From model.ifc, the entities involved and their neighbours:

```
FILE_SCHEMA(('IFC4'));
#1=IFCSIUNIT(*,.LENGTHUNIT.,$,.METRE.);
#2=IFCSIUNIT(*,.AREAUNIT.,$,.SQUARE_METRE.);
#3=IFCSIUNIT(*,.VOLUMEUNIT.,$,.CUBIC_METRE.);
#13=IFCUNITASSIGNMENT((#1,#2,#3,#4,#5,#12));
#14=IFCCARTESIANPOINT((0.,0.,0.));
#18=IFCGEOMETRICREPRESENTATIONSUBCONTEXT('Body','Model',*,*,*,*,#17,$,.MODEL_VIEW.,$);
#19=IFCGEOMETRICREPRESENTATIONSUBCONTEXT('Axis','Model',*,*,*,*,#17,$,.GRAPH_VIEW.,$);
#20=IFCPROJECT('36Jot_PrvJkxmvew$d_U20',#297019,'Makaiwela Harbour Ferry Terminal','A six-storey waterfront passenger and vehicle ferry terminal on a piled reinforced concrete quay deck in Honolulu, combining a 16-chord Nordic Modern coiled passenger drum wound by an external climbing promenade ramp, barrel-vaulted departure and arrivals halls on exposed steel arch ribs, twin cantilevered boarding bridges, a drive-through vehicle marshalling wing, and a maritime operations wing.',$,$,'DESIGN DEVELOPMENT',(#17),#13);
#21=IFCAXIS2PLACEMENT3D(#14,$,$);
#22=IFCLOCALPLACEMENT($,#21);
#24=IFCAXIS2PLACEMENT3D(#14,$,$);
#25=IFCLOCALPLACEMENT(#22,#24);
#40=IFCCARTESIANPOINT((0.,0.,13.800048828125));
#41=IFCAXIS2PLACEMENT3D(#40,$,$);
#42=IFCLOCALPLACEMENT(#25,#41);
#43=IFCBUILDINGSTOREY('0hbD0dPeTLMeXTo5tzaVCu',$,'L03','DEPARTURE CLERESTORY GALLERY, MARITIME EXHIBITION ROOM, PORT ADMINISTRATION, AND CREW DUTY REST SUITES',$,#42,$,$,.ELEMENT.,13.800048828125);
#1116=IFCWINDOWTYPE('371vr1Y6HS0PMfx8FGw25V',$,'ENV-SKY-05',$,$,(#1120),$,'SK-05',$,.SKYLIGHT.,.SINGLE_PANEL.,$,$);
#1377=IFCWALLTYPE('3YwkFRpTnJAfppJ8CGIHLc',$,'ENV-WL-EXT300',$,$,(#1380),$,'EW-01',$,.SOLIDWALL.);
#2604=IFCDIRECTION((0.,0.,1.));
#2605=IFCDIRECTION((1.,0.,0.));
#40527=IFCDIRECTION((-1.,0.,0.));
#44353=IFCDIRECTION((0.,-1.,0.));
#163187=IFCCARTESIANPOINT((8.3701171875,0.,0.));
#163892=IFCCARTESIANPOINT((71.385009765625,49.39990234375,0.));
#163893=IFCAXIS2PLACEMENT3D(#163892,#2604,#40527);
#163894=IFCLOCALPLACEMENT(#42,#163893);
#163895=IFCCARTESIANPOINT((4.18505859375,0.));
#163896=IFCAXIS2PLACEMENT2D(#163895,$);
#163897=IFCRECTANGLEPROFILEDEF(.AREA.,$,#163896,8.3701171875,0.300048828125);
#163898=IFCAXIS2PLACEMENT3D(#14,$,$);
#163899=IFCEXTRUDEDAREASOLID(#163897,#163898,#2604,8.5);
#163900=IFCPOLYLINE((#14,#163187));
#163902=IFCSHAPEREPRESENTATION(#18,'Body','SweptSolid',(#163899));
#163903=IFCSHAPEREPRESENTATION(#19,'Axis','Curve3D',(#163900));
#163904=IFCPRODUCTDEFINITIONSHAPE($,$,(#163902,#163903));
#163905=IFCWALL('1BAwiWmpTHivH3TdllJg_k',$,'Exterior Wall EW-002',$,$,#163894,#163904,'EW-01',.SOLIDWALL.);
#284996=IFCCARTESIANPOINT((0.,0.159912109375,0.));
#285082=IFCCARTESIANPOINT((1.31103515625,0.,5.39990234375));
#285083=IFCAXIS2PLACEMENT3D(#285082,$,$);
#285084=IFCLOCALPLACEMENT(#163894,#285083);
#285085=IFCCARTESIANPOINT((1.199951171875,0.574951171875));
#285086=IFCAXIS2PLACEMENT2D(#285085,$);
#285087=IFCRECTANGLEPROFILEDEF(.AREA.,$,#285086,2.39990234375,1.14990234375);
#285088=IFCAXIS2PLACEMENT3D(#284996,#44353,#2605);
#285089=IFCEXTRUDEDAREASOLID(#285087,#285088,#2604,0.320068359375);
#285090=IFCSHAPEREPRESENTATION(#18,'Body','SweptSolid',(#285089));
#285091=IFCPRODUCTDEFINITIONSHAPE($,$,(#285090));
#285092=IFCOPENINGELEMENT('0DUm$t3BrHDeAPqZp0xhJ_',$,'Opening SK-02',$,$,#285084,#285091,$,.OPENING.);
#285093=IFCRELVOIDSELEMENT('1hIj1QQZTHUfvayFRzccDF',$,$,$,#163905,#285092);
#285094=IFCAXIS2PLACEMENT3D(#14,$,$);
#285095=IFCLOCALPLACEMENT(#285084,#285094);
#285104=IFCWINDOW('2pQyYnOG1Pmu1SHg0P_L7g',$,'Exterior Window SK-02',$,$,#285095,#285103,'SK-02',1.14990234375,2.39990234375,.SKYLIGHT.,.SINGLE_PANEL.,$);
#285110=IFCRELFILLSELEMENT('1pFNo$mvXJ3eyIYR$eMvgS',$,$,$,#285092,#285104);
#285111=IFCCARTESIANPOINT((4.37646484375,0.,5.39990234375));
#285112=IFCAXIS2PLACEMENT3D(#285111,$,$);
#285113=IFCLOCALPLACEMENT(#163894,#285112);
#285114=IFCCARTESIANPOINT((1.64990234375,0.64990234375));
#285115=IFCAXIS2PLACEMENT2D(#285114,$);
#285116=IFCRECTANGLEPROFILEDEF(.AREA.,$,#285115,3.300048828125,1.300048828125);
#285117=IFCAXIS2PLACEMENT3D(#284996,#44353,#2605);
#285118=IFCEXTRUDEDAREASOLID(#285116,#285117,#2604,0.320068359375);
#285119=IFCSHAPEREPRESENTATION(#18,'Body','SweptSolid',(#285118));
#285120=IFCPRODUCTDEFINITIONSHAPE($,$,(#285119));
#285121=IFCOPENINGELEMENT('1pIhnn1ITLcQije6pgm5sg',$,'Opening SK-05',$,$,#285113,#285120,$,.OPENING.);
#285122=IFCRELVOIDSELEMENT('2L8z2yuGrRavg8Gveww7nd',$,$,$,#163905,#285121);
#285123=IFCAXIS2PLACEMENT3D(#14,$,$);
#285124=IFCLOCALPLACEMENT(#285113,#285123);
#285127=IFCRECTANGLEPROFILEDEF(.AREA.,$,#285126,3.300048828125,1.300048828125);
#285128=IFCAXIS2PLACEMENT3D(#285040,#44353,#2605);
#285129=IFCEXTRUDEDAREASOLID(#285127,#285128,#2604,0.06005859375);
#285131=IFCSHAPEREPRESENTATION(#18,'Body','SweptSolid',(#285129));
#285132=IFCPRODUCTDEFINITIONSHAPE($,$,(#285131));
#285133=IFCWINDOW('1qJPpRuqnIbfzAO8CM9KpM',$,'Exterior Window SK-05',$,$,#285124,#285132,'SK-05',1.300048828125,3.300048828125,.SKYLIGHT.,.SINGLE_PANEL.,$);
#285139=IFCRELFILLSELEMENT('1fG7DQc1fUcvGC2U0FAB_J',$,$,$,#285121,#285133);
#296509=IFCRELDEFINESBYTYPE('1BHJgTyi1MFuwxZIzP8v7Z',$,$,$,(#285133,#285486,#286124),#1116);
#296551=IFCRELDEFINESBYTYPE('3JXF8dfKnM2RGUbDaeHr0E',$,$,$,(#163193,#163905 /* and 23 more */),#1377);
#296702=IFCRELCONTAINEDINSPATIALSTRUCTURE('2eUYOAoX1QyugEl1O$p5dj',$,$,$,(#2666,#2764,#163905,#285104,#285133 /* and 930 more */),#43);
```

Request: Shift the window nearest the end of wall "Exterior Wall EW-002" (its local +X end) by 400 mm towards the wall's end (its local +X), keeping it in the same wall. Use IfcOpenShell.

```python
import ifcopenshell
import ifcopenshell.api.geometry
import ifcopenshell.util.placement
import ifcopenshell.util.unit

model = ifcopenshell.open("model.ifc")
unit_scale = ifcopenshell.util.unit.calculate_unit_scale(model)

window = model.by_id(285133)
opening = window.FillsVoids[0].RelatingOpeningElement
wall = opening.VoidsElements[0].RelatingBuildingElement

wall_matrix = ifcopenshell.util.placement.get_local_placement(wall.ObjectPlacement)
shift = wall_matrix[:3, 0] * 0.4 / unit_scale
before = ifcopenshell.util.placement.get_local_placement(window.ObjectPlacement)[:3, 3].copy()

# The window is placed relative to its opening, so it follows when the opening moves.
matrix = ifcopenshell.util.placement.get_local_placement(opening.ObjectPlacement)
matrix[:3, 3] += shift
ifcopenshell.api.geometry.edit_object_placement(
    model, product=opening, matrix=matrix, is_si=False, should_transform_children=True
)

after = ifcopenshell.util.placement.get_local_placement(window.ObjectPlacement)[:3, 3]
print("window moved by", (after - before).round(3) + 0.0)

model.write("model_updated.ifc")
```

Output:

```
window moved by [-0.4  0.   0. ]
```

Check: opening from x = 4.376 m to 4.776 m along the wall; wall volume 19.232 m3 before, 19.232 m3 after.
